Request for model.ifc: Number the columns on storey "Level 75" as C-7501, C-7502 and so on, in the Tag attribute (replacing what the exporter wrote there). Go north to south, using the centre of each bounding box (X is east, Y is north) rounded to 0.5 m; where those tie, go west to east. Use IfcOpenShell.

First a look at what the model holds.

```python
import ifcopenshell
import ifcopenshell.util.element
import ifcopenshell.util.placement

model = ifcopenshell.open("model.ifc")
print(model.schema)
storey = next(s for s in model.by_type("IfcBuildingStorey") if s.Name == "Level 75")
columns = [e for e in ifcopenshell.util.element.get_decomposition(storey) if e.is_a("IfcColumn")]
for e in sorted(columns, key=lambda e: e.id()):
    origin = ifcopenshell.util.placement.get_local_placement(e.ObjectPlacement)[:3, 3]
    print(e.id(), e.Tag, e.Name, origin.round(2) + 0.0, sep=" | ")
```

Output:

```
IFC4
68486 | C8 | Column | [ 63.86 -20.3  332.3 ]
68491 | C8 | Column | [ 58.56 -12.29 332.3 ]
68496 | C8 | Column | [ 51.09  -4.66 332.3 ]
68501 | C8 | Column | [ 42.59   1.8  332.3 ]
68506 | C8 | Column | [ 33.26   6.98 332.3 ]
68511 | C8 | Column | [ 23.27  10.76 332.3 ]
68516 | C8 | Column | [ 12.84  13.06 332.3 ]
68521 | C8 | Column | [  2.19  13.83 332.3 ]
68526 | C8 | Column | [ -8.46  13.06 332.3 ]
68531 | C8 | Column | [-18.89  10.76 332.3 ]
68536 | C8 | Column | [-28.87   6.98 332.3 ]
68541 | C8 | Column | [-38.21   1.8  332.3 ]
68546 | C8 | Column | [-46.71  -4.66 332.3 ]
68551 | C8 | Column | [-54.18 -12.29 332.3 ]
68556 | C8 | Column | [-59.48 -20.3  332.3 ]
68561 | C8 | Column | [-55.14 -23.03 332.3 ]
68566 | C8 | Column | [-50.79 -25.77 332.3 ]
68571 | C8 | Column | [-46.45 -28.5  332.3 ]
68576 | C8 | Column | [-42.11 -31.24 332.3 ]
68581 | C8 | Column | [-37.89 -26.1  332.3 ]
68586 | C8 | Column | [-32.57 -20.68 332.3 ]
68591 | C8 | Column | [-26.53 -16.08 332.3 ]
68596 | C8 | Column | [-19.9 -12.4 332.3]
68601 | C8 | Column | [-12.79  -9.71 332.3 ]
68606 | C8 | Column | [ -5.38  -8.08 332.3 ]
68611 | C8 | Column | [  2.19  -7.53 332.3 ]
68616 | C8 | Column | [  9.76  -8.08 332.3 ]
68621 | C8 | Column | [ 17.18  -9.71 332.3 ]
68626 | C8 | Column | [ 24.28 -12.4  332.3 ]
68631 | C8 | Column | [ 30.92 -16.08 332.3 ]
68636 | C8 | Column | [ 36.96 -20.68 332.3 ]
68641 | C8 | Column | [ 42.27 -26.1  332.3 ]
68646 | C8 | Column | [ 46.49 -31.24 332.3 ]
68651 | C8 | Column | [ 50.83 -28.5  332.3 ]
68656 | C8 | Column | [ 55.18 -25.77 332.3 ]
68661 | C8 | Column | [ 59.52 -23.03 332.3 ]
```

```python
import ifcopenshell
import ifcopenshell.geom
import ifcopenshell.util.element
import ifcopenshell.util.shape

model = ifcopenshell.open("model.ifc")
settings = ifcopenshell.geom.settings()
settings.set("use-world-coords", True)


def centre(element):
    shape = ifcopenshell.geom.create_shape(settings, element)
    return ifcopenshell.util.shape.get_bbox_centroid(shape.geometry)


storey = next(s for s in model.by_type("IfcBuildingStorey") if s.Name == "Level 75")
columns = [e for e in ifcopenshell.util.element.get_decomposition(storey) if e.is_a("IfcColumn")]

# Insertion points can sit at a corner or the storey origin, so sort by the geometry (in metres).
centres = {e: centre(e) for e in columns}
columns.sort(key=lambda e: (-round(centres[e][1] / 0.5), centres[e][0]))

for i, e in enumerate(columns, start=1):
    number = f"C-75{i:02d}"
    e.Tag = number
    print(e.id(), number)

model.write("model-out.ifc")
```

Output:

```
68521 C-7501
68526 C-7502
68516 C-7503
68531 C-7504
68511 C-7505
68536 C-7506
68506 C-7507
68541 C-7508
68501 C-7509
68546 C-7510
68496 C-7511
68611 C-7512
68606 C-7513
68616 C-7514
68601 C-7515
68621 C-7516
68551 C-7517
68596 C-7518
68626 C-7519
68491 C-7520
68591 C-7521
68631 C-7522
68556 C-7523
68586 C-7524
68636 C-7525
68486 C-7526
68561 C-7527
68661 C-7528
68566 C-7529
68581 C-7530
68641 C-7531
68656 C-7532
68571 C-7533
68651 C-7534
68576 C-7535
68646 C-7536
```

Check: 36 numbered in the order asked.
